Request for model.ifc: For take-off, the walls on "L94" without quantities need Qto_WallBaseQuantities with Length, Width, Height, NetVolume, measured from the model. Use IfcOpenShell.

First a look at what the model holds.

```python
import ifcopenshell
import ifcopenshell.util.element
import ifcopenshell.util.unit

model = ifcopenshell.open("model.ifc")
print(model.schema)
for unit_type in ("LENGTHUNIT", "AREAUNIT", "VOLUMEUNIT"):
    print(unit_type, ifcopenshell.util.unit.calculate_unit_scale(model, unit_type))
storey = next(s for s in model.by_type("IfcBuildingStorey") if s.Name == "L94")
walls = [e for e in ifcopenshell.util.element.get_decomposition(storey) if e.is_a("IfcWall")]
for e in sorted(walls, key=lambda e: e.id()):
    print(e.id(), e.is_a(), e.Name, list(ifcopenshell.util.element.get_psets(e, qtos_only=True)), sep=" | ")
```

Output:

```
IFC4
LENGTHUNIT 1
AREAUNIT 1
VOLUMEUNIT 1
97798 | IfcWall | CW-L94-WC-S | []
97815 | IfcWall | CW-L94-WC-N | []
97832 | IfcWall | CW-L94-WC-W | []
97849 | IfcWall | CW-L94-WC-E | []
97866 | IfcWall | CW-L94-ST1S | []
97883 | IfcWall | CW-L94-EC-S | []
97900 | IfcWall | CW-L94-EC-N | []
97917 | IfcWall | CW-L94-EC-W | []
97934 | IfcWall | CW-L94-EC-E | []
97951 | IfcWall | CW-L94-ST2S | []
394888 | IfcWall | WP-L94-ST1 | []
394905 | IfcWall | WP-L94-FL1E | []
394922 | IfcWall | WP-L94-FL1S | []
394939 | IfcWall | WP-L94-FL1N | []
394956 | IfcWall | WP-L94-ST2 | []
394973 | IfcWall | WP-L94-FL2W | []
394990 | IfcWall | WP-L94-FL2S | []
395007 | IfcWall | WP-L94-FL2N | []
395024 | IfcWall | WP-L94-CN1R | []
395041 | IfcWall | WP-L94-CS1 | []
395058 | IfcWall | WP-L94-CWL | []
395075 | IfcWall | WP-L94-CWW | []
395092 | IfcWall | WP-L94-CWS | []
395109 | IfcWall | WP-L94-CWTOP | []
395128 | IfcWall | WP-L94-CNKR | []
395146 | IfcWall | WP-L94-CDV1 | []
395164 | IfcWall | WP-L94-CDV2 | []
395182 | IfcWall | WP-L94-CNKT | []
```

```python
import ifcopenshell
import ifcopenshell.api.pset
import ifcopenshell.geom
import ifcopenshell.util.element
import ifcopenshell.util.shape
import ifcopenshell.util.unit

model = ifcopenshell.open("model.ifc")
unit_scale = ifcopenshell.util.unit.calculate_unit_scale(model)
volume_scale = ifcopenshell.util.unit.calculate_unit_scale(model, "VOLUMEUNIT")
settings = ifcopenshell.geom.settings()

storey = next(s for s in model.by_type("IfcBuildingStorey") if s.Name == "L94")
walls = [e for e in ifcopenshell.util.element.get_decomposition(storey) if e.is_a("IfcWall")]

for e in sorted(walls, key=lambda e: e.id()):
    if ifcopenshell.util.element.get_psets(e, qtos_only=True, should_inherit=False):
        continue
    # Geometry comes back in metres, in the element's own axes.
    shape = ifcopenshell.geom.create_shape(settings, e)
    values = {
        "Length": ifcopenshell.util.shape.get_x(shape.geometry) / unit_scale,
        "Width": ifcopenshell.util.shape.get_y(shape.geometry) / unit_scale,
        "Height": ifcopenshell.util.shape.get_z(shape.geometry) / unit_scale,
        "NetVolume": ifcopenshell.util.shape.get_volume(shape.geometry) / volume_scale,
    }
    qto = ifcopenshell.api.pset.add_qto(model, product=e, name="Qto_WallBaseQuantities")
    ifcopenshell.api.pset.edit_qto(model, qto=qto, properties=values)
    print(e.id(), {k: round(v, 3) for k, v in values.items()})

model.write("model_edited.ifc")
```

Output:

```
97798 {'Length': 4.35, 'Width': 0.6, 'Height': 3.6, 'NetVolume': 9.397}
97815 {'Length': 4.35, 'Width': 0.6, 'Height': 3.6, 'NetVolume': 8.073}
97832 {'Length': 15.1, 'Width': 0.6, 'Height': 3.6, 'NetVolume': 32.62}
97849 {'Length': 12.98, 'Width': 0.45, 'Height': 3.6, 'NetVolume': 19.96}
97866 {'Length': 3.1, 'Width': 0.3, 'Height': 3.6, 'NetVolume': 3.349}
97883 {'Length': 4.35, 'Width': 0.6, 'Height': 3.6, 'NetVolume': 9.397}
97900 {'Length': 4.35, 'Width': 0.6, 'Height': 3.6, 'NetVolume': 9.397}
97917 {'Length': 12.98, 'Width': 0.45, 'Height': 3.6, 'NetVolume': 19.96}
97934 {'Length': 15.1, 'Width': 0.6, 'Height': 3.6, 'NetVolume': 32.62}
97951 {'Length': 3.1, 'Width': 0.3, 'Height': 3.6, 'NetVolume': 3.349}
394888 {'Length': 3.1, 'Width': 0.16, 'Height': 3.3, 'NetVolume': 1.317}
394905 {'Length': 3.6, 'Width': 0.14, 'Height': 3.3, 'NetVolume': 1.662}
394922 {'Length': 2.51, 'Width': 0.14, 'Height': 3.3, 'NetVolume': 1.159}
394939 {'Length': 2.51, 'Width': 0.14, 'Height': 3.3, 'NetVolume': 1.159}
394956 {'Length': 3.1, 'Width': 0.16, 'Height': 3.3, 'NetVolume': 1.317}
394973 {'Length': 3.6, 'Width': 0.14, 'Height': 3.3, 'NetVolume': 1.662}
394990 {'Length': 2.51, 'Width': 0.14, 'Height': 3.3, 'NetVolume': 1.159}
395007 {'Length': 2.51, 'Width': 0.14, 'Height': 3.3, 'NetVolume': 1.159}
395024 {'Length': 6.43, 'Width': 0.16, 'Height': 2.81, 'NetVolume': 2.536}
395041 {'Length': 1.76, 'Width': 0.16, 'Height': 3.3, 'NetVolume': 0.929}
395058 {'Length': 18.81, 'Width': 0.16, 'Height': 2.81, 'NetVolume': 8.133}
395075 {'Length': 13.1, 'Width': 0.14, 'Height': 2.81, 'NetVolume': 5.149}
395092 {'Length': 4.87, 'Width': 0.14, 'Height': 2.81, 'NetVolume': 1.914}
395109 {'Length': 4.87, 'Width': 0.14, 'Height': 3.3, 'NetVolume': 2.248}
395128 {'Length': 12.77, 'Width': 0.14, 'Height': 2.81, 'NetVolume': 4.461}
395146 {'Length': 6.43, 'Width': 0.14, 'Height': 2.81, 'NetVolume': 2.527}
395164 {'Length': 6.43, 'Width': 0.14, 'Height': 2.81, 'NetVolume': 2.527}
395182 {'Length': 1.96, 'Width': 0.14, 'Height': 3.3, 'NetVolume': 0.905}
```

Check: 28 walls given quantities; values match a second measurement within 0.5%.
